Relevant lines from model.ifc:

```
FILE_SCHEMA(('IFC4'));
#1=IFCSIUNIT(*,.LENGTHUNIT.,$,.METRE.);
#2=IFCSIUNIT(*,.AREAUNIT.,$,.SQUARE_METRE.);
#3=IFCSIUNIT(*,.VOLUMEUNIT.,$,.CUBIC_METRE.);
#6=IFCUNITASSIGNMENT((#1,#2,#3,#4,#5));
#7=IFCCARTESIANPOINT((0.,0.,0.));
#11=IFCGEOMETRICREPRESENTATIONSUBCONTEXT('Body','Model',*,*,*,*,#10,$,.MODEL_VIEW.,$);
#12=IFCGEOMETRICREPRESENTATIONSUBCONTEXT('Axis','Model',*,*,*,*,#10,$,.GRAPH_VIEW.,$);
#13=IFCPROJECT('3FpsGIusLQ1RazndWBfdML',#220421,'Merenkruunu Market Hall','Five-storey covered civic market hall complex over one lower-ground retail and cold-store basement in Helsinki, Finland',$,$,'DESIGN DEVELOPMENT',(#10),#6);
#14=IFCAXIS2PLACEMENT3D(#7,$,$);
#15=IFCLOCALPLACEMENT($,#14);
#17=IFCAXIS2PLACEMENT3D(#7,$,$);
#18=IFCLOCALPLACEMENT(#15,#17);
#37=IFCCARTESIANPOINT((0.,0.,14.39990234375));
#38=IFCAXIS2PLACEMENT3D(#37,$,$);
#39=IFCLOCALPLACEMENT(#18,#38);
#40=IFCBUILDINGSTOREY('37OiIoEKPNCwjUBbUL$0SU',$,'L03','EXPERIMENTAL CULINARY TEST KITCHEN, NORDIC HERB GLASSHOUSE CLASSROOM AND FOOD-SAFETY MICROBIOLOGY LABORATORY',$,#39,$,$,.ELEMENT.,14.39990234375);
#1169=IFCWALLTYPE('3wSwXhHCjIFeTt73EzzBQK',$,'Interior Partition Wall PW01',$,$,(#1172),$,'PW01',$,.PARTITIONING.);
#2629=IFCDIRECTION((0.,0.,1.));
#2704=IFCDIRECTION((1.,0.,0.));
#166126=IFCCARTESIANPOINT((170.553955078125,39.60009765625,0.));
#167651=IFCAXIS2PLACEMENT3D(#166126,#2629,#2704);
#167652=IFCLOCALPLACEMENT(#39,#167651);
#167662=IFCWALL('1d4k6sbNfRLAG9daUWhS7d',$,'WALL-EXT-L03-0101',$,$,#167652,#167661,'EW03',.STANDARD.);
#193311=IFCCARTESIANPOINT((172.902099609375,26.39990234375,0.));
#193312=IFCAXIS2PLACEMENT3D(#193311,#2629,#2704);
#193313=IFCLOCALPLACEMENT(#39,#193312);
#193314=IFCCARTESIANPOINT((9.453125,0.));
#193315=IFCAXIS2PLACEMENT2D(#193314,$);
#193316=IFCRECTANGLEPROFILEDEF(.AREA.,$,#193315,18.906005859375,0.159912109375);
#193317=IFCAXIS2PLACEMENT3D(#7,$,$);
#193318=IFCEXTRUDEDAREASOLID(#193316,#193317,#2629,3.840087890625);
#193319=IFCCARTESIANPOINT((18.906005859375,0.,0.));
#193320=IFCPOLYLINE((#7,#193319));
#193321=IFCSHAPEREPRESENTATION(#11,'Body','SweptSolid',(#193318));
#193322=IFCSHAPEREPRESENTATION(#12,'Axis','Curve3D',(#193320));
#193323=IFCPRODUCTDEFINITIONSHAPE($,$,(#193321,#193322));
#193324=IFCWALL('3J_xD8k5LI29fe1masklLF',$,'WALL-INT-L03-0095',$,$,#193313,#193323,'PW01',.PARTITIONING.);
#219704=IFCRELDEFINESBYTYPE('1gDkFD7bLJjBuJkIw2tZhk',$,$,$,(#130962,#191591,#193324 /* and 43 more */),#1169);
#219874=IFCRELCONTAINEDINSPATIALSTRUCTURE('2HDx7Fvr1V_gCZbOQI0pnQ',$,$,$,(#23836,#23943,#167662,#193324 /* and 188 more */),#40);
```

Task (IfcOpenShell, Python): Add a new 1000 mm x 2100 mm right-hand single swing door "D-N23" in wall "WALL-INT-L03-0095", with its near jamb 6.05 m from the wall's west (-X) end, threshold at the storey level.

```python
import numpy as np
import ifcopenshell
import ifcopenshell.api.feature
import ifcopenshell.api.geometry
import ifcopenshell.api.root
import ifcopenshell.api.spatial
import ifcopenshell.geom
import ifcopenshell.util.element
import ifcopenshell.util.placement
import ifcopenshell.util.representation
import ifcopenshell.util.shape
import ifcopenshell.util.unit

model = ifcopenshell.open("model.ifc")
unit_scale = ifcopenshell.util.unit.calculate_unit_scale(model)
settings = ifcopenshell.geom.settings()


def volume(element):
    """Net volume in cubic metres, openings subtracted."""
    shape = ifcopenshell.geom.create_shape(settings, element)
    return ifcopenshell.util.shape.get_volume(shape.geometry)


wall = model.by_guid("3J_xD8k5LI29fe1masklLF")
storey = ifcopenshell.util.element.get_container(wall, ifc_class="IfcBuildingStorey")
context = ifcopenshell.util.representation.get_context(model, "Model", "Body", "MODEL_VIEW")
before = volume(wall)

width, height, from_end, sill = 1, 2.1, 6.05, 0.0  # metres

# The wall runs along its own X axis, and the end named is its -X end.
wall_shape = ifcopenshell.geom.create_shape(settings, wall)
x, y, z = ifcopenshell.util.shape.get_vertices(wall_shape.geometry).T
start = x.min() + from_end
face, thickness = float(y.min()), float(y.max() - y.min())
wall_matrix = ifcopenshell.util.placement.get_local_placement(wall.ObjectPlacement)
level = ifcopenshell.util.placement.get_local_placement(storey.ObjectPlacement)[2, 3]


def in_wall(x, y):
    """Placement at x, y metres in the wall's axes, at sill height."""
    matrix = wall_matrix.copy()
    matrix[:, 3] = wall_matrix @ np.array([x / unit_scale, y / unit_scale, 0.0, 1.0])
    matrix[2, 3] = level + sill / unit_scale
    return matrix


# Opening: a box that overshoots both wall faces by 50 mm.
opening = ifcopenshell.api.root.create_entity(model, ifc_class="IfcOpeningElement", predefined_type="OPENING")
box = ifcopenshell.api.geometry.add_wall_representation(
    model, context=context, length=width, height=height, thickness=thickness + 0.1
)
ifcopenshell.api.geometry.assign_representation(model, product=opening, representation=box)
ifcopenshell.api.geometry.edit_object_placement(model, product=opening, matrix=in_wall(start, face - 0.05), is_si=False)
ifcopenshell.api.feature.add_feature(model, feature=opening, element=wall)

door = ifcopenshell.api.root.create_entity(model, ifc_class="IfcDoor", name="D-N23", predefined_type="DOOR")
door.OverallWidth, door.OverallHeight = width / unit_scale, height / unit_scale
door.OperationType = "SINGLE_SWING_RIGHT"
body = ifcopenshell.api.geometry.add_door_representation(
    model,
    context=context,
    overall_width=door.OverallWidth,
    overall_height=door.OverallHeight,
    operation_type="SINGLE_SWING_RIGHT",
    lining_properties={"LiningDepth": thickness / unit_scale, "ThresholdDepth": thickness / unit_scale},
)
ifcopenshell.api.geometry.assign_representation(model, product=door, representation=body)
ifcopenshell.api.spatial.assign_container(model, products=[door], relating_structure=storey)
ifcopenshell.api.feature.add_filling(model, opening=opening, element=door)

# The lining spans the wall, so the door starts at the wall face.
ifcopenshell.api.geometry.edit_object_placement(model, product=door, matrix=in_wall(start, face), is_si=False)

after = volume(wall)

print(f"wall volume {before:.3f} -> {after:.3f} m3")

model.write("model-out.ifc")
```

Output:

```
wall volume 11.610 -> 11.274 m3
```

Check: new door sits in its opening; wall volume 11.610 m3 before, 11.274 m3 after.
